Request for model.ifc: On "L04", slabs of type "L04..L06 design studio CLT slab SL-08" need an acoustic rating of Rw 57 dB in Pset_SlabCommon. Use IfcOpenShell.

First a look at what the model holds.

```python
import ifcopenshell
import ifcopenshell.util.element

model = ifcopenshell.open("model.ifc")
print(model.schema)
storey = next(s for s in model.by_type("IfcBuildingStorey") if s.Name == "L04")
slabs = [e for e in ifcopenshell.util.element.get_decomposition(storey) if e.is_a("IfcSlab")]
seen = {}
for e in slabs:
    element_type = ifcopenshell.util.element.get_type(e)
    key = (element_type.Name if element_type != e and element_type else None, ifcopenshell.util.element.get_pset(e, "Pset_SlabCommon", "AcousticRating"))
    seen[key] = seen.get(key, 0) + 1
for (name, value), count in sorted(seen.items(), key=str):
    print(count, "x", name, "|", value)
```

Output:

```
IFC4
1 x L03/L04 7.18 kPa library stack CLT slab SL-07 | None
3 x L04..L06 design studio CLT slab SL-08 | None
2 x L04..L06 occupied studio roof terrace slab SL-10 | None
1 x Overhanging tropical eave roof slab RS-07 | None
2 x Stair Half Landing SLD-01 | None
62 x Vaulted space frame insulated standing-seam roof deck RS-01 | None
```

```python
import ifcopenshell
import ifcopenshell.api.pset
import ifcopenshell.util.element

model = ifcopenshell.open("model.ifc")

storey = next(s for s in model.by_type("IfcBuildingStorey") if s.Name == "L04")
slabs = [e for e in ifcopenshell.util.element.get_decomposition(storey) if e.is_a("IfcSlab")]

count = 0
for e in slabs:
    element_type = ifcopenshell.util.element.get_type(e)
    if element_type in (None, e) or element_type.Name != "L04..L06 design studio CLT slab SL-08":
        continue
    # add_pset returns the element's existing set when there is one.
    pset = ifcopenshell.api.pset.add_pset(model, product=e, name="Pset_SlabCommon")
    ifcopenshell.api.pset.edit_pset(model, pset=pset, properties={"AcousticRating": "Rw 57 dB"})
    count += 1

print(count, "slabs updated")

model.write("model-out.ifc")
```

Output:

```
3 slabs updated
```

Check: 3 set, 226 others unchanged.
